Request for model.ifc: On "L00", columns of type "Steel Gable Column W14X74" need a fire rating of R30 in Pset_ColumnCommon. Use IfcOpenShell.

First a look at what the model holds.

```python
import ifcopenshell
import ifcopenshell.util.element

model = ifcopenshell.open("model.ifc")
print(model.schema)
storey = next(s for s in model.by_type("IfcBuildingStorey") if s.Name == "L00")
columns = [e for e in ifcopenshell.util.element.get_decomposition(storey) if e.is_a("IfcColumn")]
seen = {}
for e in columns:
    element_type = ifcopenshell.util.element.get_type(e)
    key = (element_type.Name if element_type != e and element_type else None, ifcopenshell.util.element.get_pset(e, "Pset_ColumnCommon", "FireRating"))
    seen[key] = seen.get(key, 0) + 1
for (name, value), count in sorted(seen.items(), key=str):
    print(count, "x", name, "|", value)
```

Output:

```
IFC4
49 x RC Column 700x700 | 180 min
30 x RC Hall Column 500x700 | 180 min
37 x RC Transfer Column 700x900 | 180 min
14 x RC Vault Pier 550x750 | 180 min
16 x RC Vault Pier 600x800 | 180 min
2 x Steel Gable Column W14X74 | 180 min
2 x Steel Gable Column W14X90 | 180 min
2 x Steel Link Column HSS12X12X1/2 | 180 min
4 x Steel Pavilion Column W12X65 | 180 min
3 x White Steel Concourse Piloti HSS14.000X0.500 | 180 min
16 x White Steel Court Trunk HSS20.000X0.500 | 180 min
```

```python
import ifcopenshell
import ifcopenshell.api.pset
import ifcopenshell.util.element

model = ifcopenshell.open("model.ifc")

storey = next(s for s in model.by_type("IfcBuildingStorey") if s.Name == "L00")
columns = [e for e in ifcopenshell.util.element.get_decomposition(storey) if e.is_a("IfcColumn")]

count = 0
for e in columns:
    element_type = ifcopenshell.util.element.get_type(e)
    if element_type in (None, e) or element_type.Name != "Steel Gable Column W14X74":
        continue
    # add_pset returns the element's existing set when there is one.
    pset = ifcopenshell.api.pset.add_pset(model, product=e, name="Pset_ColumnCommon")
    ifcopenshell.api.pset.edit_pset(model, pset=pset, properties={"FireRating": "R30"})
    count += 1

print(count, "columns updated")

model.write("model_v2.ifc")
```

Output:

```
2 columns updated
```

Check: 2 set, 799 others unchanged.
